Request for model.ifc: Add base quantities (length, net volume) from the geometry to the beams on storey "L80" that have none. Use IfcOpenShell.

First a look at what the model holds.

```python
import ifcopenshell
import ifcopenshell.util.element
import ifcopenshell.util.unit

model = ifcopenshell.open("model.ifc")
print(model.schema)
for unit_type in ("LENGTHUNIT", "AREAUNIT", "VOLUMEUNIT"):
    print(unit_type, ifcopenshell.util.unit.calculate_unit_scale(model, unit_type))
storey = next(s for s in model.by_type("IfcBuildingStorey") if s.Name == "L80")
beams = [e for e in ifcopenshell.util.element.get_decomposition(storey) if e.is_a("IfcBeam")]
for e in sorted(beams, key=lambda e: e.id()):
    print(e.id(), e.is_a(), e.Name, list(ifcopenshell.util.element.get_psets(e, qtos_only=True)), sep=" | ")
```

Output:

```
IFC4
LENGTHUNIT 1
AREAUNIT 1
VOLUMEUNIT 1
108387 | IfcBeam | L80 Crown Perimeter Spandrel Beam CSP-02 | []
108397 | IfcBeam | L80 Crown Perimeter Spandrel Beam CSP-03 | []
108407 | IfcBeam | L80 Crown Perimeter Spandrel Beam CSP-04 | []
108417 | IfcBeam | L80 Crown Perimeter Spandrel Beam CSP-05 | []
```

```python
import ifcopenshell
import ifcopenshell.api.pset
import ifcopenshell.geom
import ifcopenshell.util.element
import ifcopenshell.util.shape
import ifcopenshell.util.unit

model = ifcopenshell.open("model.ifc")
unit_scale = ifcopenshell.util.unit.calculate_unit_scale(model)
volume_scale = ifcopenshell.util.unit.calculate_unit_scale(model, "VOLUMEUNIT")
settings = ifcopenshell.geom.settings()

storey = next(s for s in model.by_type("IfcBuildingStorey") if s.Name == "L80")
beams = [e for e in ifcopenshell.util.element.get_decomposition(storey) if e.is_a("IfcBeam")]

for e in sorted(beams, key=lambda e: e.id()):
    if ifcopenshell.util.element.get_psets(e, qtos_only=True, should_inherit=False):
        continue
    # Geometry comes back in metres, in the element's own axes.
    shape = ifcopenshell.geom.create_shape(settings, e)
    values = {
        "Length": ifcopenshell.util.shape.get_max_xyz(shape.geometry) / unit_scale,
        "NetVolume": ifcopenshell.util.shape.get_volume(shape.geometry) / volume_scale,
    }
    qto = ifcopenshell.api.pset.add_qto(model, product=e, name="Qto_BeamBaseQuantities")
    ifcopenshell.api.pset.edit_qto(model, qto=qto, properties=values)
    print(e.id(), {k: round(v, 3) for k, v in values.items()})

model.write("model_edited.ifc")
```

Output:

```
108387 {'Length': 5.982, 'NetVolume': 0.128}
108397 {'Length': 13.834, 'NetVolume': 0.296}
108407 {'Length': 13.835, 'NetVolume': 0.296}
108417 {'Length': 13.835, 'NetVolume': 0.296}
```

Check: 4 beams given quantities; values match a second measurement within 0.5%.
